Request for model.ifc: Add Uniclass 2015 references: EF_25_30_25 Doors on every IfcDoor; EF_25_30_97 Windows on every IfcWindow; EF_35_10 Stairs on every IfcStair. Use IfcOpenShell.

First a look at what the model holds.

```python
import ifcopenshell

model = ifcopenshell.open("model.ifc")
print(model.schema)
print("classifications:", [c.Name for c in model.by_type("IfcClassification")])
for ifc_class in ("IfcDoor", "IfcRoof", "IfcStair", "IfcWall", "IfcWindow"):
    print(ifc_class, len(model.by_type(ifc_class)))
```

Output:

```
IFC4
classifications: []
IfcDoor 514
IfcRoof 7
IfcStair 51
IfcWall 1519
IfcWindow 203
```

```python
import ifcopenshell
import ifcopenshell.api.classification

model = ifcopenshell.open("model.ifc")

system = ifcopenshell.api.classification.add_classification(model, classification="Uniclass 2015")

codes = {
    "IfcDoor": ("EF_25_30_25", "Doors"),
    "IfcWindow": ("EF_25_30_97", "Windows"),
    "IfcStair": ("EF_35_10", "Stairs"),
}
for ifc_class, (code, name) in codes.items():
    products = model.by_type(ifc_class)
    ifcopenshell.api.classification.add_reference(
        model, products=products, classification=system, identification=code, name=name
    )
    print(code, len(products))

model.write("model_v2.ifc")
```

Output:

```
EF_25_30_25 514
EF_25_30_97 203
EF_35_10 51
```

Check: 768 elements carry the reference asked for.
